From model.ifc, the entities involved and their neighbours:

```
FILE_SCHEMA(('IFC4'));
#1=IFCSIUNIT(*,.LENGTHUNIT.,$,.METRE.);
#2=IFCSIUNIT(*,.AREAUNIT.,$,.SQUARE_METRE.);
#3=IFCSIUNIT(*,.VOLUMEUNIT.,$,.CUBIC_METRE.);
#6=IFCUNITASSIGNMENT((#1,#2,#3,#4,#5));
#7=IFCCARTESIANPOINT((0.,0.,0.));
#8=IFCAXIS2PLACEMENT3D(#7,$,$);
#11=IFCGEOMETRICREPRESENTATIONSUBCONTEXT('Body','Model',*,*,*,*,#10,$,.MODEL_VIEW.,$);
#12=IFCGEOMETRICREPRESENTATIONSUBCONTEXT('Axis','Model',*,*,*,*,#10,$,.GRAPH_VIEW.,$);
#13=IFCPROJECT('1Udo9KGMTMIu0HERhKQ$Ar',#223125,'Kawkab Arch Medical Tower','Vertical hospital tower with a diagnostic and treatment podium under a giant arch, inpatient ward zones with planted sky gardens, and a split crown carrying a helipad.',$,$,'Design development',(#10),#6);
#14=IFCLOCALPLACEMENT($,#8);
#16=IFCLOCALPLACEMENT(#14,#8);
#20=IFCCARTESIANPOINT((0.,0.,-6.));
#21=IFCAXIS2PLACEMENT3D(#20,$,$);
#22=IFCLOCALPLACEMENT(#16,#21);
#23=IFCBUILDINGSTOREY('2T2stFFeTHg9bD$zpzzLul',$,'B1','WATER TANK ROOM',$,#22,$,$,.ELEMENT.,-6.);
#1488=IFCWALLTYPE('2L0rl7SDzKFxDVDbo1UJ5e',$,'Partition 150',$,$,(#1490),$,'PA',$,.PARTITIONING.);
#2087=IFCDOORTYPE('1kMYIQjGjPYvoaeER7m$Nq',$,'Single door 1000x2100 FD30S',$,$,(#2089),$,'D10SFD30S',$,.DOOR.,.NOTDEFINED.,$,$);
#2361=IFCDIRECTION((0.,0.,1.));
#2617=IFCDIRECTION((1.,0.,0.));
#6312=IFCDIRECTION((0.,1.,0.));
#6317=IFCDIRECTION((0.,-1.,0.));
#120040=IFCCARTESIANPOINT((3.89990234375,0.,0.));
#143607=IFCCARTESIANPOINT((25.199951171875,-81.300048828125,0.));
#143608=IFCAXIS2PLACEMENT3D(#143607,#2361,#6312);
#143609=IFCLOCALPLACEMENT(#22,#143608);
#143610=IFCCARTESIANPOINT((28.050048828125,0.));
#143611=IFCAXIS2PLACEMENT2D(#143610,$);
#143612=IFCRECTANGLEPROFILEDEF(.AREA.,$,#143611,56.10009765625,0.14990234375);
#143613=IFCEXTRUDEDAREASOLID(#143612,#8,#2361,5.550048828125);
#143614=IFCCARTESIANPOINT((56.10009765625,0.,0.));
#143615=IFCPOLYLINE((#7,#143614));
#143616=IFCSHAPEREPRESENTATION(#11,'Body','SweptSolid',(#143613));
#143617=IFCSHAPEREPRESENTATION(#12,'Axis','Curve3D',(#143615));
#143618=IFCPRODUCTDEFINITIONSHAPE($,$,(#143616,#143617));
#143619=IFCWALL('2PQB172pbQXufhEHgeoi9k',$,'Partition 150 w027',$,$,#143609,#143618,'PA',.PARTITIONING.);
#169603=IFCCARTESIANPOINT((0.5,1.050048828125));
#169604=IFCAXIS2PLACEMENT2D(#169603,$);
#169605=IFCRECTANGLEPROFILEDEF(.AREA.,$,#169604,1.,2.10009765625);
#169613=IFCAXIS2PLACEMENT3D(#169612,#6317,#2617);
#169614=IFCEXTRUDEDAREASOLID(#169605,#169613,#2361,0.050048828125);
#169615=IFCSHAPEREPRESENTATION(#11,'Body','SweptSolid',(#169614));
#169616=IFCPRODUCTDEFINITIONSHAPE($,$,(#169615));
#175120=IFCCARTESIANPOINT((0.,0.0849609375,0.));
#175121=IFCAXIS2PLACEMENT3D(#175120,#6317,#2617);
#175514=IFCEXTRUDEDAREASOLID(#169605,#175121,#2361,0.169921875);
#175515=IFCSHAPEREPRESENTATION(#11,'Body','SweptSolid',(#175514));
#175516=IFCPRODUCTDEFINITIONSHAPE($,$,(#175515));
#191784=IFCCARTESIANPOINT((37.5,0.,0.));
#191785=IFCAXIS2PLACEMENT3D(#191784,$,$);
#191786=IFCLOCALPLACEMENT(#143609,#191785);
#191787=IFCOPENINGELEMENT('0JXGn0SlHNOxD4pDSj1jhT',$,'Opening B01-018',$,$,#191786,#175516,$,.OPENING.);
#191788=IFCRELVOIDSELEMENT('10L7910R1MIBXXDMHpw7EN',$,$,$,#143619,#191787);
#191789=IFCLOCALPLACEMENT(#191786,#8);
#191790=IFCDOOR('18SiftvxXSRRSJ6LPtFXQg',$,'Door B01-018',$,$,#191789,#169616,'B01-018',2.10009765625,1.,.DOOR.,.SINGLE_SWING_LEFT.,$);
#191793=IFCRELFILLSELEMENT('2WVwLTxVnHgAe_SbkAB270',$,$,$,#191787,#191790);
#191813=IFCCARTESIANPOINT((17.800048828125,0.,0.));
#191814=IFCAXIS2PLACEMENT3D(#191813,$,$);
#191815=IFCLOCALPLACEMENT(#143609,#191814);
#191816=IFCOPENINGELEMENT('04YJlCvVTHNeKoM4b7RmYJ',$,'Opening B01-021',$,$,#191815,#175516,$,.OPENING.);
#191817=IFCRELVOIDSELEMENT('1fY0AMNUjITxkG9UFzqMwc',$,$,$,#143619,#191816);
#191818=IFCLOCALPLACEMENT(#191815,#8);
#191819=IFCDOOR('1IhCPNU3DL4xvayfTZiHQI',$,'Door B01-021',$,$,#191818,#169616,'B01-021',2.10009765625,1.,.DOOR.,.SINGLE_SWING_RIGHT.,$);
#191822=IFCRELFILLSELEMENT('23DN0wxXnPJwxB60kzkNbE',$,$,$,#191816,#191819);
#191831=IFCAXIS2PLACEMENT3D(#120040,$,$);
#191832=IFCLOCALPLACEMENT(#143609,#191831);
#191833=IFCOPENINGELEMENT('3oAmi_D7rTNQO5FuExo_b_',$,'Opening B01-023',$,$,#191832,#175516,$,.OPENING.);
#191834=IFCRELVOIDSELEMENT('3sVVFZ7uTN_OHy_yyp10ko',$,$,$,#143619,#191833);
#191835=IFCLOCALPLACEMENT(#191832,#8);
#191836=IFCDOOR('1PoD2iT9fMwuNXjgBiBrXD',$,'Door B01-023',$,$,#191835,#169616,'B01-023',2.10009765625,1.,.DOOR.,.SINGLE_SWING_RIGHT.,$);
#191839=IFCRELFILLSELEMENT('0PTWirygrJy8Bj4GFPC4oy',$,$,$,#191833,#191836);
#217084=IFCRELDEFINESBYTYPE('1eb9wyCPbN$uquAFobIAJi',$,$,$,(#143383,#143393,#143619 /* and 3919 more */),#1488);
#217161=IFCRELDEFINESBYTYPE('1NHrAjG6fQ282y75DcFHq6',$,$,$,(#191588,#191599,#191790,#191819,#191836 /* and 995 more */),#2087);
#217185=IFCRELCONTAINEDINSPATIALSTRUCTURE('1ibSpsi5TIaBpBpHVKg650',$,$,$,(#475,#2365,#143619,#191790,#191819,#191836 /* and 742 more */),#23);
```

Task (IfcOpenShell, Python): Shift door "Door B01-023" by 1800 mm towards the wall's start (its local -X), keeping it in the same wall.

```python
import ifcopenshell
import ifcopenshell.api.geometry
import ifcopenshell.util.placement
import ifcopenshell.util.unit

model = ifcopenshell.open("model.ifc")
unit_scale = ifcopenshell.util.unit.calculate_unit_scale(model)

door = model.by_id(191836)
opening = door.FillsVoids[0].RelatingOpeningElement
wall = opening.VoidsElements[0].RelatingBuildingElement

wall_matrix = ifcopenshell.util.placement.get_local_placement(wall.ObjectPlacement)
shift = wall_matrix[:3, 0] * -1.8 / unit_scale
before = ifcopenshell.util.placement.get_local_placement(door.ObjectPlacement)[:3, 3].copy()

# The door is placed relative to its opening, so it follows when the opening moves.
matrix = ifcopenshell.util.placement.get_local_placement(opening.ObjectPlacement)
matrix[:3, 3] += shift
ifcopenshell.api.geometry.edit_object_placement(
    model, product=opening, matrix=matrix, is_si=False, should_transform_children=True
)

after = ifcopenshell.util.placement.get_local_placement(door.ObjectPlacement)[:3, 3]
print("door moved by", (after - before).round(3) + 0.0)

model.write("model_edited.ifc")
```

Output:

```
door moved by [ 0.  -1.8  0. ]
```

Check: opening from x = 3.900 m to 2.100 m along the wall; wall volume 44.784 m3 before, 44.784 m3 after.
